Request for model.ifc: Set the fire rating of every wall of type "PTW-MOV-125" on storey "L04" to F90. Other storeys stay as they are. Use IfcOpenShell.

First a look at what the model holds.

```python
import ifcopenshell
import ifcopenshell.util.element

model = ifcopenshell.open("model.ifc")
print(model.schema)
storey = next(s for s in model.by_type("IfcBuildingStorey") if s.Name == "L04")
walls = [e for e in ifcopenshell.util.element.get_decomposition(storey) if e.is_a("IfcWall")]
seen = {}
for e in walls:
    element_type = ifcopenshell.util.element.get_type(e)
    key = (element_type.Name if element_type != e and element_type else None, ifcopenshell.util.element.get_pset(e, "Pset_WallCommon", "FireRating"))
    seen[key] = seen.get(key, 0) + 1
for (name, value), count in sorted(seen.items(), key=str):
    print(count, "x", name, "|", value)
```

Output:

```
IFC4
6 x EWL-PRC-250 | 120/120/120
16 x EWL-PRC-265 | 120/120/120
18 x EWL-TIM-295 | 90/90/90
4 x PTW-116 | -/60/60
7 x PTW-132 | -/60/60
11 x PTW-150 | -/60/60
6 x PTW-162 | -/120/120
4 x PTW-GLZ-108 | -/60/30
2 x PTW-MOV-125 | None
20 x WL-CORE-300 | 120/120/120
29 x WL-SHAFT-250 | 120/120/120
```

```python
import ifcopenshell
import ifcopenshell.api.pset
import ifcopenshell.util.element

model = ifcopenshell.open("model.ifc")

storey = next(s for s in model.by_type("IfcBuildingStorey") if s.Name == "L04")
walls = [e for e in ifcopenshell.util.element.get_decomposition(storey) if e.is_a("IfcWall")]

count = 0
for e in walls:
    element_type = ifcopenshell.util.element.get_type(e)
    if element_type in (None, e) or element_type.Name != "PTW-MOV-125":
        continue
    # add_pset returns the element's existing set when there is one.
    pset = ifcopenshell.api.pset.add_pset(model, product=e, name="Pset_WallCommon")
    ifcopenshell.api.pset.edit_pset(model, pset=pset, properties={"FireRating": "F90"})
    count += 1

print(count, "walls updated")

model.write("model_v2.ifc")
```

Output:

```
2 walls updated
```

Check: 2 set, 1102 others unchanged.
